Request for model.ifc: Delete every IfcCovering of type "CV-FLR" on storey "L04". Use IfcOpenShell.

First a look at what the model holds.

```python
import ifcopenshell
import ifcopenshell.util.element

model = ifcopenshell.open("model.ifc")
print(model.schema)
storey = next(s for s in model.by_type("IfcBuildingStorey") if s.Name == "L04")
coverings = [e for e in ifcopenshell.util.element.get_decomposition(storey) if e.is_a("IfcCovering")]
seen = {}
for e in coverings:
    element_type = ifcopenshell.util.element.get_type(e)
    name = element_type.Name if element_type not in (None, e) else None
    seen[name] = seen.get(name, 0) + 1
for name, count in sorted(seen.items(), key=str):
    print(count, "x", name)
```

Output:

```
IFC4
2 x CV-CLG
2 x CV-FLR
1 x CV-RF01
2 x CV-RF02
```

```python
import ifcopenshell
import ifcopenshell.api.root
import ifcopenshell.util.element

model = ifcopenshell.open("model.ifc")

storey = next(s for s in model.by_type("IfcBuildingStorey") if s.Name == "L04")
coverings = [e for e in ifcopenshell.util.element.get_decomposition(storey) if e.is_a("IfcCovering")]
targets = [e for e in coverings if (t := ifcopenshell.util.element.get_type(e)) not in (None, e) and t.Name == "CV-FLR"]

for e in targets:
    ifcopenshell.api.root.remove_product(model, product=e)
print(len(targets), "removed")

model.write("model_v2.ifc")
```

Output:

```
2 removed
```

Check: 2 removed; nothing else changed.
